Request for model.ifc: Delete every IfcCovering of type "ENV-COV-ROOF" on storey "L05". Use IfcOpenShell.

First a look at what the model holds.

```python
import ifcopenshell
import ifcopenshell.util.element

model = ifcopenshell.open("model.ifc")
print(model.schema)
storey = next(s for s in model.by_type("IfcBuildingStorey") if s.Name == "L05")
coverings = [e for e in ifcopenshell.util.element.get_decomposition(storey) if e.is_a("IfcCovering")]
seen = {}
for e in coverings:
    element_type = ifcopenshell.util.element.get_type(e)
    name = element_type.Name if element_type not in (None, e) else None
    seen[name] = seen.get(name, 0) + 1
for name, count in sorted(seen.items(), key=str):
    print(count, "x", name)
```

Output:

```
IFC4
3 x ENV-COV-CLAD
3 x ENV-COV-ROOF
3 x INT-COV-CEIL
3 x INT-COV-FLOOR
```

```python
import ifcopenshell
import ifcopenshell.api.root
import ifcopenshell.util.element

model = ifcopenshell.open("model.ifc")

storey = next(s for s in model.by_type("IfcBuildingStorey") if s.Name == "L05")
coverings = [e for e in ifcopenshell.util.element.get_decomposition(storey) if e.is_a("IfcCovering")]
targets = [e for e in coverings if (t := ifcopenshell.util.element.get_type(e)) not in (None, e) and t.Name == "ENV-COV-ROOF"]

for e in targets:
    ifcopenshell.api.root.remove_product(model, product=e)
print(len(targets), "removed")

model.write("model_v2.ifc")
```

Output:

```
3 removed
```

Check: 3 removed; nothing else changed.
